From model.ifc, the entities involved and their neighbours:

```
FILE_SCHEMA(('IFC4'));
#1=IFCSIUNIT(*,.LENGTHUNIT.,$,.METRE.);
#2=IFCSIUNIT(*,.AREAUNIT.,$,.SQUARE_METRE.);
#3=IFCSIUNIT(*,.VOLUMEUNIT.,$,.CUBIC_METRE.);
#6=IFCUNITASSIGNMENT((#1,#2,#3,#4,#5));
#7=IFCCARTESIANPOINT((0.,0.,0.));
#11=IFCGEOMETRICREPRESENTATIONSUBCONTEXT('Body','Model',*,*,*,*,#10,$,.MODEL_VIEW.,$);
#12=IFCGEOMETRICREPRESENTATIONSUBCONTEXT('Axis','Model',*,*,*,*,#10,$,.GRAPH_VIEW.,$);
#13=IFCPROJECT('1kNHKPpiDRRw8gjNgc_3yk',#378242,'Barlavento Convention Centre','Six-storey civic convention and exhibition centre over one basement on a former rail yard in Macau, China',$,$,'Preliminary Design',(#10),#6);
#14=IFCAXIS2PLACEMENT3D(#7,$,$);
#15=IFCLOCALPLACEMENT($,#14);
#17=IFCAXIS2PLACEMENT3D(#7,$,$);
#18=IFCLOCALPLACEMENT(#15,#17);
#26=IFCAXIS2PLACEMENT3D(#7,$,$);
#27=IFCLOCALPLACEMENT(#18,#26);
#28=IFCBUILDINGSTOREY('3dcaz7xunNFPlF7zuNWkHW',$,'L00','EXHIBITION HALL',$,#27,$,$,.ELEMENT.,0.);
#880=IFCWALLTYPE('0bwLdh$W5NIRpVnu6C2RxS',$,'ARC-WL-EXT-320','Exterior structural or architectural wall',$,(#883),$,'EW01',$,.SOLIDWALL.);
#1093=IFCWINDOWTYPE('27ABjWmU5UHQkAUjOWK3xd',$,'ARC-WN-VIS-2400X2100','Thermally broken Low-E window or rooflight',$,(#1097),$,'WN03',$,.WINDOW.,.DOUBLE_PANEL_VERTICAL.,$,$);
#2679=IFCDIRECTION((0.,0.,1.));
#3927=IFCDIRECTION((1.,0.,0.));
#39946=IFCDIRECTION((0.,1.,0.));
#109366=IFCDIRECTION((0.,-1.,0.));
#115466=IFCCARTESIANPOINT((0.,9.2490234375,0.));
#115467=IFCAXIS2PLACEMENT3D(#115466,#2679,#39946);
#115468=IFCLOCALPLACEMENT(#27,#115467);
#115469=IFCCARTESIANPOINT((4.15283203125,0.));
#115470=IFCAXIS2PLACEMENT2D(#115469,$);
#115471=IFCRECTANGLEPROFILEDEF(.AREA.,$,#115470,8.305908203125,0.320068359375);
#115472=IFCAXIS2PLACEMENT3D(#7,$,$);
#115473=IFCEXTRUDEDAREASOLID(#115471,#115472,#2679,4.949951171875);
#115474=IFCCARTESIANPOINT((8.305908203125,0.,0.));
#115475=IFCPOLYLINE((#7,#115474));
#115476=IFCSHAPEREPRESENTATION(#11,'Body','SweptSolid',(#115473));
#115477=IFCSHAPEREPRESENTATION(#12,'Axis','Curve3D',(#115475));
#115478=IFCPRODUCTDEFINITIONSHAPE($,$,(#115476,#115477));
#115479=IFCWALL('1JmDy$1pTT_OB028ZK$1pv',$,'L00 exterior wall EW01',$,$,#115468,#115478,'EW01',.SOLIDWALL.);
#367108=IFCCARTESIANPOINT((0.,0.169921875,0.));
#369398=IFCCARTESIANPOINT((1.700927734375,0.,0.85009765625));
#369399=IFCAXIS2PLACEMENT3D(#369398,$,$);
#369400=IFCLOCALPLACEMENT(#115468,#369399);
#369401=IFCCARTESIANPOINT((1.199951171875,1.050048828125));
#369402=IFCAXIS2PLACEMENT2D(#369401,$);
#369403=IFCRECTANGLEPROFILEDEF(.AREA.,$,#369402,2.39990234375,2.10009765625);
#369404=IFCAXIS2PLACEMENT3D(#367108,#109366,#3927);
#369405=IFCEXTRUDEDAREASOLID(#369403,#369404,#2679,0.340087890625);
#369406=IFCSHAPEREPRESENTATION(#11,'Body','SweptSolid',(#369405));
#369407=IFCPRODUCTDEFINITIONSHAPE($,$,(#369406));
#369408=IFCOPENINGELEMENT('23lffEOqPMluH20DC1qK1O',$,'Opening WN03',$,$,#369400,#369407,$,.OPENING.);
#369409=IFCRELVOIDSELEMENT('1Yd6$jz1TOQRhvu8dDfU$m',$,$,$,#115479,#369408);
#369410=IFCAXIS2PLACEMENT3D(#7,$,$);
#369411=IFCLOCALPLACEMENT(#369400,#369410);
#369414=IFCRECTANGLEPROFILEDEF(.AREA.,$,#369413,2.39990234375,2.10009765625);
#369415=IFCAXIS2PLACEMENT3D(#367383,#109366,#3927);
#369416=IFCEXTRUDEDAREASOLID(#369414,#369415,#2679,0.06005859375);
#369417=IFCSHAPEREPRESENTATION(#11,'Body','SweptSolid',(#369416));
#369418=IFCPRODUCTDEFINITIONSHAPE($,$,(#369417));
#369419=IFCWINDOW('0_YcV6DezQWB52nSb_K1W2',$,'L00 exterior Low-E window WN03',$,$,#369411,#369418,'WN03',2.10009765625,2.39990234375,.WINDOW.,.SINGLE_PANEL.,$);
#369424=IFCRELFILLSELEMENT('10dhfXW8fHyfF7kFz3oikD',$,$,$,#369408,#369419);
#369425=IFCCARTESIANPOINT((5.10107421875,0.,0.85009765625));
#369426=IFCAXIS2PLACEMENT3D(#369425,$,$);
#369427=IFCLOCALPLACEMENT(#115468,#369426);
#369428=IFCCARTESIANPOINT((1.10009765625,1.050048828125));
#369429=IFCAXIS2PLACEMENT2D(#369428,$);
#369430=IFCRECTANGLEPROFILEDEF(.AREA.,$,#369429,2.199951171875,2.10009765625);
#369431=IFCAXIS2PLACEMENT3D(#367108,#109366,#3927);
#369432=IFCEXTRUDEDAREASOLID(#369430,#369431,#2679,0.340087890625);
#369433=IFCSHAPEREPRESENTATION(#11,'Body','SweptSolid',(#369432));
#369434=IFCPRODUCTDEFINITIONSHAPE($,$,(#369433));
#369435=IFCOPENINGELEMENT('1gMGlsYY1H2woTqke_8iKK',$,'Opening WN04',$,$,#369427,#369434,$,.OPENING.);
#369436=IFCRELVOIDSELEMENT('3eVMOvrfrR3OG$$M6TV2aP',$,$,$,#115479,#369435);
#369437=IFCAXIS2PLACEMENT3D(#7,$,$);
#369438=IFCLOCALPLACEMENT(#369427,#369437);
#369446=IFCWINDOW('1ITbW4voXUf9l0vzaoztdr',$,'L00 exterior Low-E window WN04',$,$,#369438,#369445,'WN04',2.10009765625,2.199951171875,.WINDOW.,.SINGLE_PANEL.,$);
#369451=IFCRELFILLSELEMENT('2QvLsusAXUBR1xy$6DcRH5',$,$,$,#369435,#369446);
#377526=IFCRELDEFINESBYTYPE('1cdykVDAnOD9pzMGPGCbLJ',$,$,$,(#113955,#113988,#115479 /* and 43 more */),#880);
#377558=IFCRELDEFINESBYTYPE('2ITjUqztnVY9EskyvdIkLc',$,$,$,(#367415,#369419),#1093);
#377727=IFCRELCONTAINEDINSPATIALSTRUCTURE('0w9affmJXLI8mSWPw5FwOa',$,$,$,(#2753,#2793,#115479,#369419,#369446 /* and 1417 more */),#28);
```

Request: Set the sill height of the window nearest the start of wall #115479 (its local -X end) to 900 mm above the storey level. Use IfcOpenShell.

```python
import numpy as np
import ifcopenshell
import ifcopenshell.api.geometry
import ifcopenshell.geom
import ifcopenshell.util.element
import ifcopenshell.util.placement
import ifcopenshell.util.shape
import ifcopenshell.util.unit

model = ifcopenshell.open("model.ifc")
unit_scale = ifcopenshell.util.unit.calculate_unit_scale(model)

window = model.by_id(369419)
opening = window.FillsVoids[0].RelatingOpeningElement
storey = ifcopenshell.util.element.get_container(window, ifc_class="IfcBuildingStorey")
level = ifcopenshell.util.placement.get_local_placement(storey.ObjectPlacement)[2, 3]

# The opening's origin need not be at the sill, so measure its lowest point.
shape = ifcopenshell.geom.create_shape(ifcopenshell.geom.settings(), opening)
bottom = ifcopenshell.util.shape.get_shape_bottom_elevation(shape, shape.geometry) / unit_scale
dz = level + 0.9 / unit_scale - bottom

shift = np.array([0.0, 0.0, dz])
# The window is placed relative to its opening, so it follows when the opening moves.
matrix = ifcopenshell.util.placement.get_local_placement(opening.ObjectPlacement)
matrix[:3, 3] += shift
ifcopenshell.api.geometry.edit_object_placement(
    model, product=opening, matrix=matrix, is_si=False, should_transform_children=True
)

print(f"moved by {dz * unit_scale:+.3f} m")

model.write("model-out.ifc")
```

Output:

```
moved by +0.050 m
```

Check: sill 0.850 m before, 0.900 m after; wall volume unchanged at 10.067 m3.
